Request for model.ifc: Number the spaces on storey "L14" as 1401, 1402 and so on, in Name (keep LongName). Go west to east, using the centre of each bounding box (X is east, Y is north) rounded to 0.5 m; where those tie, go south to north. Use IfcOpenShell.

First a look at what the model holds.

```python
import ifcopenshell
import ifcopenshell.util.element
import ifcopenshell.util.placement

model = ifcopenshell.open("model.ifc")
print(model.schema)
storey = next(s for s in model.by_type("IfcBuildingStorey") if s.Name == "L14")
spaces = [e for e in ifcopenshell.util.element.get_decomposition(storey) if e.is_a("IfcSpace")]
for e in sorted(spaces, key=lambda e: e.id()):
    origin = ifcopenshell.util.placement.get_local_placement(e.ObjectPlacement)[:3, 3]
    print(e.id(), e.Name, e.LongName, origin.round(2) + 0.0, sep=" | ")
```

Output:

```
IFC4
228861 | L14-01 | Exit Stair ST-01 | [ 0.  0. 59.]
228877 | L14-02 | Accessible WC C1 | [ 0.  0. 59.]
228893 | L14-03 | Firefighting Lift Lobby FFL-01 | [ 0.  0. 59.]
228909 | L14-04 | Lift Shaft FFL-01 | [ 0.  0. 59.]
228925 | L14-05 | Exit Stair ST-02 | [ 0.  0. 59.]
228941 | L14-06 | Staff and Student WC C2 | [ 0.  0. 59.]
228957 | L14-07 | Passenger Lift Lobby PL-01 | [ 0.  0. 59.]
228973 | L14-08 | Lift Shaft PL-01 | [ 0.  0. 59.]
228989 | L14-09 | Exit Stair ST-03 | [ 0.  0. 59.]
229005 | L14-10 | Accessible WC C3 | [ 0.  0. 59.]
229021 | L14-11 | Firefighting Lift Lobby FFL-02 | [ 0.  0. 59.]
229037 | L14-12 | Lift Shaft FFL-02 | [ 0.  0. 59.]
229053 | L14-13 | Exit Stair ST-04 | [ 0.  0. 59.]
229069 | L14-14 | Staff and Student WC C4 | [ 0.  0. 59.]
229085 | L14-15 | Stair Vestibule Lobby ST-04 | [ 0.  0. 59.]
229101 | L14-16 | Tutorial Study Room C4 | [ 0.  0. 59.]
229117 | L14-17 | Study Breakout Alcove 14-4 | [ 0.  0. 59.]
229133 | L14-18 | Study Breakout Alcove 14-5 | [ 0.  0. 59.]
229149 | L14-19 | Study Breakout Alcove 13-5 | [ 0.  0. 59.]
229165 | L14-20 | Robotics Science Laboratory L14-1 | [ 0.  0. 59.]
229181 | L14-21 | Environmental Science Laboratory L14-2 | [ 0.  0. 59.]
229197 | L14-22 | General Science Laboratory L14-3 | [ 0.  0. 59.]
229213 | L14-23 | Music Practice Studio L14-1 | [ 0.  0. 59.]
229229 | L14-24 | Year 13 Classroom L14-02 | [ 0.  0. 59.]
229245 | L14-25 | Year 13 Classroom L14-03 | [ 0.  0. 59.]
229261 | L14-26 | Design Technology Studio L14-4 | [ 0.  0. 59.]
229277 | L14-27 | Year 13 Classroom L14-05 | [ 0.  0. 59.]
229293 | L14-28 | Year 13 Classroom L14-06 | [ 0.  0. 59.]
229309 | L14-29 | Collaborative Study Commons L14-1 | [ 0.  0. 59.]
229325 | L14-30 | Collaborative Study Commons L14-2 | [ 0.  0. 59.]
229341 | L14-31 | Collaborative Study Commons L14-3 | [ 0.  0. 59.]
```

```python
import ifcopenshell
import ifcopenshell.geom
import ifcopenshell.util.element
import ifcopenshell.util.shape

model = ifcopenshell.open("model.ifc")
settings = ifcopenshell.geom.settings()
settings.set("use-world-coords", True)


def centre(element):
    shape = ifcopenshell.geom.create_shape(settings, element)
    return ifcopenshell.util.shape.get_bbox_centroid(shape.geometry)


storey = next(s for s in model.by_type("IfcBuildingStorey") if s.Name == "L14")
spaces = [e for e in ifcopenshell.util.element.get_decomposition(storey) if e.is_a("IfcSpace")]

# Insertion points can sit at a corner or the storey origin, so sort by the geometry (in metres).
centres = {e: centre(e) for e in spaces}
spaces.sort(key=lambda e: (round(centres[e][0] / 0.5), centres[e][1]))

for i, e in enumerate(spaces, start=1):
    number = f"14{i:02d}"
    e.Name = number
    print(e.id(), number)

model.write("model_updated.ifc")
```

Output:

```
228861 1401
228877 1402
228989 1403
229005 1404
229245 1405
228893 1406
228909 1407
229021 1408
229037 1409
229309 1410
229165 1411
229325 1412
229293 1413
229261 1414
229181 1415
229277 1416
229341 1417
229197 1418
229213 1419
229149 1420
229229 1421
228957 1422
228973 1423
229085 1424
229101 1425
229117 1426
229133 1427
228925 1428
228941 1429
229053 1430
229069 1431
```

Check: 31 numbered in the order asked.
